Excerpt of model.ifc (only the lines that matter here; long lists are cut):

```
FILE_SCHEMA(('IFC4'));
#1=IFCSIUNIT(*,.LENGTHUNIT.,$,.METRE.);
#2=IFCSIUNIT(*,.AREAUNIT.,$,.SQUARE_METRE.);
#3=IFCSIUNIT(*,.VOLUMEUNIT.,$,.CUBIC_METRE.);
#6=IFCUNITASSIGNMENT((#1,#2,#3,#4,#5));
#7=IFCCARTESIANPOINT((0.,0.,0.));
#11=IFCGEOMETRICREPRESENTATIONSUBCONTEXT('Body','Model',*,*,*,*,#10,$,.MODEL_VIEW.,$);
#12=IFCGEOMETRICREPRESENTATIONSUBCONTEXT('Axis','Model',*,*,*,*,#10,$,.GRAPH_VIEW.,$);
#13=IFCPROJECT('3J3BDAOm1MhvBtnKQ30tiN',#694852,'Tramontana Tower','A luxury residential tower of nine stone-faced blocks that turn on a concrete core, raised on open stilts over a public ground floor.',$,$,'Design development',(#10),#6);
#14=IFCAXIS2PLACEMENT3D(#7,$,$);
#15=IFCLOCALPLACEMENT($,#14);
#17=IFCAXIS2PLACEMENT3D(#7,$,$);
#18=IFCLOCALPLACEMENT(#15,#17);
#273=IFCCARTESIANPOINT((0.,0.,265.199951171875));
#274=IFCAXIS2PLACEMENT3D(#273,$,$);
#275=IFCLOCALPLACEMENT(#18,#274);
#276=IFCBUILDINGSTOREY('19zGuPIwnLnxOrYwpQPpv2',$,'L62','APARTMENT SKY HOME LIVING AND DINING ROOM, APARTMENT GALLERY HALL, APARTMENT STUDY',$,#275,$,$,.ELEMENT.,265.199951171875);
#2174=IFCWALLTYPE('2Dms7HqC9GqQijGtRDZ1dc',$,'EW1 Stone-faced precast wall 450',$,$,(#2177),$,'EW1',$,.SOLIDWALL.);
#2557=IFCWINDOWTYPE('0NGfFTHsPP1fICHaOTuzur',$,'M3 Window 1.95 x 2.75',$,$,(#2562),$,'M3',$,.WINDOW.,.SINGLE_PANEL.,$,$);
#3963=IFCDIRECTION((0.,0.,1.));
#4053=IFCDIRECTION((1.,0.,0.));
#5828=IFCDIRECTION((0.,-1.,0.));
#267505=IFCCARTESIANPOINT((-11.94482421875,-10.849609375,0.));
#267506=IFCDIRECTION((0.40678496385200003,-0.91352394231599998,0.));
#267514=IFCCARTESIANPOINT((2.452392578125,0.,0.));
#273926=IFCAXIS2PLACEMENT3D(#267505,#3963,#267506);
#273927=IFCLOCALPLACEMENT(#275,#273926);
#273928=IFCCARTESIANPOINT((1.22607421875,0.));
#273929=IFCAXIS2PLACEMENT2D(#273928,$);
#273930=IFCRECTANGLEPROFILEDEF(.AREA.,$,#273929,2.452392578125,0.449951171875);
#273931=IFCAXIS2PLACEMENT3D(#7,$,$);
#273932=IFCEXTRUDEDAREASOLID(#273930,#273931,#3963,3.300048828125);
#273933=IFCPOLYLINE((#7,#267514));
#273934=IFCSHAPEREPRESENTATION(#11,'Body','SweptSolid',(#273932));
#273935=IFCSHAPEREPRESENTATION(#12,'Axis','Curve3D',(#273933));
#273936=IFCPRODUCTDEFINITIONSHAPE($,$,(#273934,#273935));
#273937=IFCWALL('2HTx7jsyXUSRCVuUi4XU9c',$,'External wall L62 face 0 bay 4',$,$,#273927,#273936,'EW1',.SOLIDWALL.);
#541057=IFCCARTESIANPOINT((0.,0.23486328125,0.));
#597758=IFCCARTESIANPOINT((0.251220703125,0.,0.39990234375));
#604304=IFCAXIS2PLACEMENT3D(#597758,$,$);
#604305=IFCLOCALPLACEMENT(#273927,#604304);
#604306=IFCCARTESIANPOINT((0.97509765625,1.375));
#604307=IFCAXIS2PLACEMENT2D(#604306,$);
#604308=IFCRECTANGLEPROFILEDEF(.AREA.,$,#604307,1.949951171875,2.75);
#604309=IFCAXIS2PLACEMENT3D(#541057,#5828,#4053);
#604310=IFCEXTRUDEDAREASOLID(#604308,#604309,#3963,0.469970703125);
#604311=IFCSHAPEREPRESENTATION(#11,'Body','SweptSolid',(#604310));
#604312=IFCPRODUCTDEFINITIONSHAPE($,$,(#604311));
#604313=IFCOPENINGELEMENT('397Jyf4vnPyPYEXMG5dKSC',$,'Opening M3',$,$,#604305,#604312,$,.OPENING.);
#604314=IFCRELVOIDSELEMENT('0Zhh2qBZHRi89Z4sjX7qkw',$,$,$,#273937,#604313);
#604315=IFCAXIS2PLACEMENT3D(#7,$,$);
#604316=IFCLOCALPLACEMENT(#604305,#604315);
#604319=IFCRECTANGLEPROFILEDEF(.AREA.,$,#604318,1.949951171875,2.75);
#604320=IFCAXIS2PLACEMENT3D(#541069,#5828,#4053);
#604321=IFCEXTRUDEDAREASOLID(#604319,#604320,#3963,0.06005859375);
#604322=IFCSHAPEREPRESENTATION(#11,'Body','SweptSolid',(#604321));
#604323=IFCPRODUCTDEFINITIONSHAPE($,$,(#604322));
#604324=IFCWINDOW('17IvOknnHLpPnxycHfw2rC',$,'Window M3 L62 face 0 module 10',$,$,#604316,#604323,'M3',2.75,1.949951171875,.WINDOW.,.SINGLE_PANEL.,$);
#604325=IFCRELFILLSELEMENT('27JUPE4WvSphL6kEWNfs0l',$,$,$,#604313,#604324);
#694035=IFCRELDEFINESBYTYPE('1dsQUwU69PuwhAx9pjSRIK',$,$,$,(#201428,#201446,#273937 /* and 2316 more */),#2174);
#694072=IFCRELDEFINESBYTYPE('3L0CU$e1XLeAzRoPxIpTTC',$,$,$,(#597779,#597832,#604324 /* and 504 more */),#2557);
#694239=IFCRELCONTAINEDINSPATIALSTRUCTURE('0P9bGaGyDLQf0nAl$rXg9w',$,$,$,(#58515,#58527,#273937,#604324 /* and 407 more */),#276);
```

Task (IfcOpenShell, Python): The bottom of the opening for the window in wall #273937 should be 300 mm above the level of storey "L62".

```python
import numpy as np
import ifcopenshell
import ifcopenshell.api.geometry
import ifcopenshell.geom
import ifcopenshell.util.element
import ifcopenshell.util.placement
import ifcopenshell.util.shape
import ifcopenshell.util.unit

model = ifcopenshell.open("model.ifc")
unit_scale = ifcopenshell.util.unit.calculate_unit_scale(model)

window = model.by_guid("17IvOknnHLpPnxycHfw2rC")
opening = window.FillsVoids[0].RelatingOpeningElement
storey = ifcopenshell.util.element.get_container(window, ifc_class="IfcBuildingStorey")
level = ifcopenshell.util.placement.get_local_placement(storey.ObjectPlacement)[2, 3]

# The opening's origin need not be at the sill, so measure its lowest point.
shape = ifcopenshell.geom.create_shape(ifcopenshell.geom.settings(), opening)
bottom = ifcopenshell.util.shape.get_shape_bottom_elevation(shape, shape.geometry) / unit_scale
dz = level + 0.3 - bottom

shift = np.array([0.0, 0.0, dz])
# The window is placed relative to its opening, so it follows when the opening moves.
matrix = ifcopenshell.util.placement.get_local_placement(opening.ObjectPlacement)
matrix[:3, 3] += shift
ifcopenshell.api.geometry.edit_object_placement(
    model, product=opening, matrix=matrix, is_si=False, should_transform_children=True
)

print(f"moved by {dz * unit_scale:+.3f} m")

model.write("model_edited.ifc")
```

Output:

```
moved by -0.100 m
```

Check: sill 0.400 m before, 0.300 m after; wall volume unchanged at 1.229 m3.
